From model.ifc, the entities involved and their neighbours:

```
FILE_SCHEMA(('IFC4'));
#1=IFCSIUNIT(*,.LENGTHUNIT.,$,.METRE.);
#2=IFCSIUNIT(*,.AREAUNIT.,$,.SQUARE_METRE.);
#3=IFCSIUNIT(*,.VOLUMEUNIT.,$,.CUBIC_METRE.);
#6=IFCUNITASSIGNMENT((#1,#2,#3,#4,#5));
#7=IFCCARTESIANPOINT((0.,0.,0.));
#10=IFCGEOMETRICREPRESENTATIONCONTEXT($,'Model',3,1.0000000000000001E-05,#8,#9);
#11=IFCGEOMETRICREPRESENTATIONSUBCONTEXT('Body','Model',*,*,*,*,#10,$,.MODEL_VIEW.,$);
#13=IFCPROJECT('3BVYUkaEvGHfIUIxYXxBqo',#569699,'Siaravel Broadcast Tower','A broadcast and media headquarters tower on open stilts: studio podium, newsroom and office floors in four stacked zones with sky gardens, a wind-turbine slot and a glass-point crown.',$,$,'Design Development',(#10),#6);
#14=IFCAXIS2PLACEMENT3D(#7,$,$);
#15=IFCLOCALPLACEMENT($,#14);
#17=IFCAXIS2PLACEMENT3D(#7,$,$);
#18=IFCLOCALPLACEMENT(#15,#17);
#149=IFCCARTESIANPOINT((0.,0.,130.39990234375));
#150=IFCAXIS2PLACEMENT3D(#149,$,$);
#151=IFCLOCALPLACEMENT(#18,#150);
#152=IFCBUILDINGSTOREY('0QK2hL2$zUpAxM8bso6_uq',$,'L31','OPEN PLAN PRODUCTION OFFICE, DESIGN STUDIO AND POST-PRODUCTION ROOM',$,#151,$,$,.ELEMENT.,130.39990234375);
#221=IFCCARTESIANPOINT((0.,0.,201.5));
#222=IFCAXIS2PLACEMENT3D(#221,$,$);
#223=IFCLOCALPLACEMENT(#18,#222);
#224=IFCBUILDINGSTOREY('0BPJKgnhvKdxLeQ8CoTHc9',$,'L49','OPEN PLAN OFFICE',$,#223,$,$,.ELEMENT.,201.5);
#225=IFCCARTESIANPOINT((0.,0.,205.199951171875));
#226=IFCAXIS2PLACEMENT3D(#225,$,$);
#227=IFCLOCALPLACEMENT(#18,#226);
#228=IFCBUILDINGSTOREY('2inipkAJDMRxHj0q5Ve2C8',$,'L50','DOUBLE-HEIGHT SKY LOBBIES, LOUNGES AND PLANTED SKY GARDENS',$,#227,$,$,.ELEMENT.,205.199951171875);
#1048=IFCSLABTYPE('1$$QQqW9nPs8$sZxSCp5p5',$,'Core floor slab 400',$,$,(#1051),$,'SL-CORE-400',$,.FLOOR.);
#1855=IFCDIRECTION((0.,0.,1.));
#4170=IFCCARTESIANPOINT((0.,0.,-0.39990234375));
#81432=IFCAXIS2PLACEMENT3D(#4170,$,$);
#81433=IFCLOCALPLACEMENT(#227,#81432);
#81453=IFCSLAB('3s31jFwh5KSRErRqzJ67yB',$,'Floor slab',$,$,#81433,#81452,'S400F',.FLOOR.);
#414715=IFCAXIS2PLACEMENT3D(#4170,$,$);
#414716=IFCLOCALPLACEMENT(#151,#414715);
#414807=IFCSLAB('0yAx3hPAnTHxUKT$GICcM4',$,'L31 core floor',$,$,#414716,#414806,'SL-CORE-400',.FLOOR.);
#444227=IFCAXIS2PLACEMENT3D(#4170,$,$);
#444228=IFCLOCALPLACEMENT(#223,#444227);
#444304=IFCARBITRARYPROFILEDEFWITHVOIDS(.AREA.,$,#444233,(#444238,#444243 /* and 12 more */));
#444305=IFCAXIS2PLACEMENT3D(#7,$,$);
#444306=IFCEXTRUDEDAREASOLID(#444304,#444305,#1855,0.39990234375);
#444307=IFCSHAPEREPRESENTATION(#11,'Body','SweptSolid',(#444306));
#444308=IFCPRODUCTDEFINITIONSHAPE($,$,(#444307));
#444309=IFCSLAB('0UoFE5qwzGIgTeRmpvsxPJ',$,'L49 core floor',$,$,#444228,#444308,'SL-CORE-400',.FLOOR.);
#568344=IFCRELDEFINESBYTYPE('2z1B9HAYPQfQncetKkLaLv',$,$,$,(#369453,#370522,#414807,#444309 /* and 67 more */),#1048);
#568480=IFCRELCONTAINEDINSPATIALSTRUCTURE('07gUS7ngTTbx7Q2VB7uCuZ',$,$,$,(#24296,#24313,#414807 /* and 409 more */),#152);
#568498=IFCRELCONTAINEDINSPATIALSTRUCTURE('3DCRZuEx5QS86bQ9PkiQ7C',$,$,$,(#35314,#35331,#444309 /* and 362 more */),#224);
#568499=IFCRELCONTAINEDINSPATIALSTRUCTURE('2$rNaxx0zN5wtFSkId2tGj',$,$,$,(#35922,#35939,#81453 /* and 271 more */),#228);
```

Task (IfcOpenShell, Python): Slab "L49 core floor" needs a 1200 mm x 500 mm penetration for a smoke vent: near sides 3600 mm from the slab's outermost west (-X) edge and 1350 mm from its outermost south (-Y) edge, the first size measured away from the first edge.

```python
import numpy as np
import ifcopenshell
import ifcopenshell.api.feature
import ifcopenshell.api.geometry
import ifcopenshell.api.root
import ifcopenshell.geom
import ifcopenshell.util.placement
import ifcopenshell.util.representation
import ifcopenshell.util.shape
import ifcopenshell.util.unit

model = ifcopenshell.open("model.ifc")
unit_scale = ifcopenshell.util.unit.calculate_unit_scale(model)
settings = ifcopenshell.geom.settings()


def volume(element):
    """Net volume in cubic metres, openings subtracted."""
    shape = ifcopenshell.geom.create_shape(settings, element)
    return ifcopenshell.util.shape.get_volume(shape.geometry)


slab = model.by_guid("0UoFE5qwzGIgTeRmpvsxPJ")
before = volume(slab)

# Extent in the slab's own axes, in metres. The edges named are its -X and -Y sides.
slab_shape = ifcopenshell.geom.create_shape(settings, slab)
vertices = ifcopenshell.util.shape.get_vertices(slab_shape.geometry)
x_min, y_min, bottom = vertices.min(axis=0)
top = vertices[:, 2].max()

opening = ifcopenshell.api.root.create_entity(model, ifc_class="IfcOpeningElement", name="Smoke vent opening", predefined_type="OPENING")
context = ifcopenshell.util.representation.get_context(model, "Model", "Body", "MODEL_VIEW")
width, depth = 1.2, 0.5
outline = [(0.0, 0.0), (width, 0.0), (width, depth), (0.0, depth), (0.0, 0.0)]
# Overshoot both faces by 50 mm so the cut is clean.
shape = ifcopenshell.api.geometry.add_slab_representation(
    model, context=context, depth=top - bottom + 0.1, polyline=outline
)
ifcopenshell.api.geometry.assign_representation(model, product=opening, representation=shape)

matrix = ifcopenshell.util.placement.get_local_placement(slab.ObjectPlacement)
matrix[:, 3] = matrix @ np.append(np.array([x_min + 3.6, y_min + 1.35, bottom - 0.05]) / unit_scale, 1.0)
ifcopenshell.api.geometry.edit_object_placement(model, product=opening, matrix=matrix, is_si=False)
ifcopenshell.api.feature.add_feature(model, feature=opening, element=slab)

after = volume(slab)

print(f"slab volume {before:.3f} -> {after:.3f} m3")

model.write("model_v2.ifc")
```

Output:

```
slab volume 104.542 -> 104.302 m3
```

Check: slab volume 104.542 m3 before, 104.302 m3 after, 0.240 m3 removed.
